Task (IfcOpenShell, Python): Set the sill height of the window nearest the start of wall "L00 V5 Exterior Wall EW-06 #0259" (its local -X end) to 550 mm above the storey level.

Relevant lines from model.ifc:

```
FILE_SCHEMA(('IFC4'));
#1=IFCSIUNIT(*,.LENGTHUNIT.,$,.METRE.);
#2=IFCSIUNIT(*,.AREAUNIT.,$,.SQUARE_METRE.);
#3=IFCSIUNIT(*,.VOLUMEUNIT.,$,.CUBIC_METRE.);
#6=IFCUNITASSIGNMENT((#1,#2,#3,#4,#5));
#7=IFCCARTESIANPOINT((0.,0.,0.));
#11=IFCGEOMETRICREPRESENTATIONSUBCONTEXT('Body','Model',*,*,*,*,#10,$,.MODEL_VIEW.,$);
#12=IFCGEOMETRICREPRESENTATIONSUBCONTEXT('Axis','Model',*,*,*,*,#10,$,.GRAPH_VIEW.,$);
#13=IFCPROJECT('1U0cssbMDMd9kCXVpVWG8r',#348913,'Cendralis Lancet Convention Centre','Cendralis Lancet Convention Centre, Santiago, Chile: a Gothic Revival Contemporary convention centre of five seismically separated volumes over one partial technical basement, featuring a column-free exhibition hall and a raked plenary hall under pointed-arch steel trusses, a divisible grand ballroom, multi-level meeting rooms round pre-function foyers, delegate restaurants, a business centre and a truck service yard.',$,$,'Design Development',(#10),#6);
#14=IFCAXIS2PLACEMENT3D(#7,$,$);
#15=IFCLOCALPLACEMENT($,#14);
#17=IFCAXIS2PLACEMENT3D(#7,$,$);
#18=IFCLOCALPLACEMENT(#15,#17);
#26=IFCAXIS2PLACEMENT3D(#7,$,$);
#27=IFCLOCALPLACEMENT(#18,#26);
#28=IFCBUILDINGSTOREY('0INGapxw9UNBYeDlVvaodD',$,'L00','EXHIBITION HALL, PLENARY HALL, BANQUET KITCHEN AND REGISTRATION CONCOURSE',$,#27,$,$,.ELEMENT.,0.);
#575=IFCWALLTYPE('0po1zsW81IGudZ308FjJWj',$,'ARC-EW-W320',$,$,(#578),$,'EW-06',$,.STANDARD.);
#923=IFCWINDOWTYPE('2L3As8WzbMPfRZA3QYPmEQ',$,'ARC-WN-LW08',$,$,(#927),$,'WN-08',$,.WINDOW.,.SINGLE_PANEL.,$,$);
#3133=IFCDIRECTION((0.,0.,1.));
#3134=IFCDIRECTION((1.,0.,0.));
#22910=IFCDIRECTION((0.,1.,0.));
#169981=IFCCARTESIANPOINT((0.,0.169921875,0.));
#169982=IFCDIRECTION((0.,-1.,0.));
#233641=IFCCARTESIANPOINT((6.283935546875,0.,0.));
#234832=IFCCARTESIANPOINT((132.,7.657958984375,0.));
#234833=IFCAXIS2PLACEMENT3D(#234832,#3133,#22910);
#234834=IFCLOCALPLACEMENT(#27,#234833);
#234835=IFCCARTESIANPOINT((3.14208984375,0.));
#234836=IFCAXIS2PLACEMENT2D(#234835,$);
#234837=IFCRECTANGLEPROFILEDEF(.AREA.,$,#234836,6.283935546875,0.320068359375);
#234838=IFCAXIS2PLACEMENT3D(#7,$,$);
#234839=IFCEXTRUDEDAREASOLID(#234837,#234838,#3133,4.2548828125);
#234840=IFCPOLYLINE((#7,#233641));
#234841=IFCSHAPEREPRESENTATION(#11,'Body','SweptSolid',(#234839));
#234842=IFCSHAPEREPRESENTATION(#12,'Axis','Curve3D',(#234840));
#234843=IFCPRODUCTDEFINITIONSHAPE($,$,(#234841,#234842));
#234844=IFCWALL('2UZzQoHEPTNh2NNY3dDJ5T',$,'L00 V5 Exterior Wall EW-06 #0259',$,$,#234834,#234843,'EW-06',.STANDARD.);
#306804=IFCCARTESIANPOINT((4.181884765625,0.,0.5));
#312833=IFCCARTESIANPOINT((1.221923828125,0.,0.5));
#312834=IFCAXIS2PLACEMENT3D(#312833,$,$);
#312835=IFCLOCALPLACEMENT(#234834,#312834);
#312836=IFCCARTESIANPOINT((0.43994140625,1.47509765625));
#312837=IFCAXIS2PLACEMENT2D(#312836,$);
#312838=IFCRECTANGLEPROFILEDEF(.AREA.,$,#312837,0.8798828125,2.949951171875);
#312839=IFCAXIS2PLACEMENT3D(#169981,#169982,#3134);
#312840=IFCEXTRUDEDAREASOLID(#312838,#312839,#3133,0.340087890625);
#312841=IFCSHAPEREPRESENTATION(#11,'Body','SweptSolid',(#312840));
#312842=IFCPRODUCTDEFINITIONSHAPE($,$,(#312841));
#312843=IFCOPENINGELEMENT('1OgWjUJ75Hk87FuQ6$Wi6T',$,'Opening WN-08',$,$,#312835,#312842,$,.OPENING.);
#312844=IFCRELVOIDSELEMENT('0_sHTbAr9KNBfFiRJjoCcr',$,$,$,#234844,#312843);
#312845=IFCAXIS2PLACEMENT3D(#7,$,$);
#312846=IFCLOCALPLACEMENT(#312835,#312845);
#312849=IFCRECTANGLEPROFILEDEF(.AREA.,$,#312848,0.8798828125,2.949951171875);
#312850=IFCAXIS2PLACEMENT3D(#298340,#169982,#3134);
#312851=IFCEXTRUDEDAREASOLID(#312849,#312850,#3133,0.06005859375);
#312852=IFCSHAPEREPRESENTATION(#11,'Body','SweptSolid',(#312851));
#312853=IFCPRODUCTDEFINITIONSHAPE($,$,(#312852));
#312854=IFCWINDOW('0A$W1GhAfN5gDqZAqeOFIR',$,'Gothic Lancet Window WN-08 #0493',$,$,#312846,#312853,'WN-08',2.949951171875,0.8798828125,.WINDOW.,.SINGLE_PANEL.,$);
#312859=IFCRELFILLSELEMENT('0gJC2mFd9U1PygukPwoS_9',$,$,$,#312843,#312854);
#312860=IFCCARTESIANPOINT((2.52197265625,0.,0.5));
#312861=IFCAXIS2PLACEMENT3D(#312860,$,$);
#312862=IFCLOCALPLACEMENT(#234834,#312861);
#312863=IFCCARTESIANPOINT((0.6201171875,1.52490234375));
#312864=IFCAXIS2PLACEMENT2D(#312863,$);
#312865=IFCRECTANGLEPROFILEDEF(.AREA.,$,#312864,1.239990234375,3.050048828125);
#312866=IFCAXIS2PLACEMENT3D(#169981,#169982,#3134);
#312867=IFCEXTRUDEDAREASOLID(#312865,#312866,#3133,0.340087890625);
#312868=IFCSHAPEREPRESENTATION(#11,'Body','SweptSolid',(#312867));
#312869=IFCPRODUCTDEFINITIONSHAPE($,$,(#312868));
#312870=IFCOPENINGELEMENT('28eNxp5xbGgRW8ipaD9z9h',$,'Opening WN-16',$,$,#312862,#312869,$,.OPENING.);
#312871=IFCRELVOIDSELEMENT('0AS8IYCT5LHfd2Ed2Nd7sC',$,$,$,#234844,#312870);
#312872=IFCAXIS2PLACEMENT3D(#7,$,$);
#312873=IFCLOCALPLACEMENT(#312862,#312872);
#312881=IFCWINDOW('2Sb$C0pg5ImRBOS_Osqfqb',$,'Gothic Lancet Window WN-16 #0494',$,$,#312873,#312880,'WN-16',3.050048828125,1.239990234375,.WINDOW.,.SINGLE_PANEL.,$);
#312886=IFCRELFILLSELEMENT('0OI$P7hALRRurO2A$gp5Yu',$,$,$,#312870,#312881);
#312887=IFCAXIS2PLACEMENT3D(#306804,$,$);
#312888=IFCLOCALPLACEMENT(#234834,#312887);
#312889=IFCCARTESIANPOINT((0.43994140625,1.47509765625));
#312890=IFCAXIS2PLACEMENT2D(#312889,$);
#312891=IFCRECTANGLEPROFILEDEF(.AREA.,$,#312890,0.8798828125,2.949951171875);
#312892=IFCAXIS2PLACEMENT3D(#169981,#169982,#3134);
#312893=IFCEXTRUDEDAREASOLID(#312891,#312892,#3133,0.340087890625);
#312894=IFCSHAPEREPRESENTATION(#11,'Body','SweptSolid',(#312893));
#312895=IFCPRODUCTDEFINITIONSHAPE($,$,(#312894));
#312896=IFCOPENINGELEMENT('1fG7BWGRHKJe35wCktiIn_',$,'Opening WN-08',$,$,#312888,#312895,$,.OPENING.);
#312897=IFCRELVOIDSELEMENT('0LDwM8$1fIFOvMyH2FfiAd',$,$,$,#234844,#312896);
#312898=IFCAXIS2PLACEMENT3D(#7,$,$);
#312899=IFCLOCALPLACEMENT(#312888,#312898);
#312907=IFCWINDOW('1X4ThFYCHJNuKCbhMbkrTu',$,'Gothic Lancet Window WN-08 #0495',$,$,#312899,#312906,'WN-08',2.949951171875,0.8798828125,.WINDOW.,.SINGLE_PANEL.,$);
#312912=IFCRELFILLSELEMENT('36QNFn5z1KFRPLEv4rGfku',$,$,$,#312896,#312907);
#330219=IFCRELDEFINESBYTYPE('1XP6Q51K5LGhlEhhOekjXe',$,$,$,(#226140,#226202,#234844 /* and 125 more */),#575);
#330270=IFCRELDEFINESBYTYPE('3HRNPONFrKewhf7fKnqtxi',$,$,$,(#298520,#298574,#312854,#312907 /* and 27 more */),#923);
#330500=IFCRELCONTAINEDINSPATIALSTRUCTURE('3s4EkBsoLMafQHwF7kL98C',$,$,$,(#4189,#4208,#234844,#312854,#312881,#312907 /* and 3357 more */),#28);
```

```python
import numpy as np
import ifcopenshell
import ifcopenshell.api.geometry
import ifcopenshell.geom
import ifcopenshell.util.element
import ifcopenshell.util.placement
import ifcopenshell.util.shape
import ifcopenshell.util.unit

model = ifcopenshell.open("model.ifc")
unit_scale = ifcopenshell.util.unit.calculate_unit_scale(model)

window = model.by_guid("0A$W1GhAfN5gDqZAqeOFIR")
opening = window.FillsVoids[0].RelatingOpeningElement
storey = ifcopenshell.util.element.get_container(window, ifc_class="IfcBuildingStorey")
level = ifcopenshell.util.placement.get_local_placement(storey.ObjectPlacement)[2, 3]

# The opening's origin need not be at the sill, so measure its lowest point.
shape = ifcopenshell.geom.create_shape(ifcopenshell.geom.settings(), opening)
bottom = ifcopenshell.util.shape.get_shape_bottom_elevation(shape, shape.geometry) / unit_scale
dz = level + 0.55 / unit_scale - bottom

shift = np.array([0.0, 0.0, dz])
# The window is placed relative to its opening, so it follows when the opening moves.
matrix = ifcopenshell.util.placement.get_local_placement(opening.ObjectPlacement)
matrix[:3, 3] += shift
ifcopenshell.api.geometry.edit_object_placement(
    model, product=opening, matrix=matrix, is_si=False, should_transform_children=True
)

print(f"moved by {dz * unit_scale:+.3f} m")

model.write("model_updated.ifc")
```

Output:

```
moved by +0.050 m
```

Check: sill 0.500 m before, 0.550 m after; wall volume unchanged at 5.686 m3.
